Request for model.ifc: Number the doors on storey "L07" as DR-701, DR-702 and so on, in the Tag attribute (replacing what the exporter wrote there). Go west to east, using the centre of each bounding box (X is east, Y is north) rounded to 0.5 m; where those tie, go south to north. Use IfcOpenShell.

First a look at what the model holds.

```python
import ifcopenshell
import ifcopenshell.util.element
import ifcopenshell.util.placement

model = ifcopenshell.open("model.ifc")
print(model.schema)
storey = next(s for s in model.by_type("IfcBuildingStorey") if s.Name == "L07")
doors = [e for e in ifcopenshell.util.element.get_decomposition(storey) if e.is_a("IfcDoor")]
for e in sorted(doors, key=lambda e: e.id()):
    origin = ifcopenshell.util.placement.get_local_placement(e.ObjectPlacement)[:3, 3]
    print(e.id(), e.Tag, e.Name, origin.round(2) + 0.0, sep=" | ")
```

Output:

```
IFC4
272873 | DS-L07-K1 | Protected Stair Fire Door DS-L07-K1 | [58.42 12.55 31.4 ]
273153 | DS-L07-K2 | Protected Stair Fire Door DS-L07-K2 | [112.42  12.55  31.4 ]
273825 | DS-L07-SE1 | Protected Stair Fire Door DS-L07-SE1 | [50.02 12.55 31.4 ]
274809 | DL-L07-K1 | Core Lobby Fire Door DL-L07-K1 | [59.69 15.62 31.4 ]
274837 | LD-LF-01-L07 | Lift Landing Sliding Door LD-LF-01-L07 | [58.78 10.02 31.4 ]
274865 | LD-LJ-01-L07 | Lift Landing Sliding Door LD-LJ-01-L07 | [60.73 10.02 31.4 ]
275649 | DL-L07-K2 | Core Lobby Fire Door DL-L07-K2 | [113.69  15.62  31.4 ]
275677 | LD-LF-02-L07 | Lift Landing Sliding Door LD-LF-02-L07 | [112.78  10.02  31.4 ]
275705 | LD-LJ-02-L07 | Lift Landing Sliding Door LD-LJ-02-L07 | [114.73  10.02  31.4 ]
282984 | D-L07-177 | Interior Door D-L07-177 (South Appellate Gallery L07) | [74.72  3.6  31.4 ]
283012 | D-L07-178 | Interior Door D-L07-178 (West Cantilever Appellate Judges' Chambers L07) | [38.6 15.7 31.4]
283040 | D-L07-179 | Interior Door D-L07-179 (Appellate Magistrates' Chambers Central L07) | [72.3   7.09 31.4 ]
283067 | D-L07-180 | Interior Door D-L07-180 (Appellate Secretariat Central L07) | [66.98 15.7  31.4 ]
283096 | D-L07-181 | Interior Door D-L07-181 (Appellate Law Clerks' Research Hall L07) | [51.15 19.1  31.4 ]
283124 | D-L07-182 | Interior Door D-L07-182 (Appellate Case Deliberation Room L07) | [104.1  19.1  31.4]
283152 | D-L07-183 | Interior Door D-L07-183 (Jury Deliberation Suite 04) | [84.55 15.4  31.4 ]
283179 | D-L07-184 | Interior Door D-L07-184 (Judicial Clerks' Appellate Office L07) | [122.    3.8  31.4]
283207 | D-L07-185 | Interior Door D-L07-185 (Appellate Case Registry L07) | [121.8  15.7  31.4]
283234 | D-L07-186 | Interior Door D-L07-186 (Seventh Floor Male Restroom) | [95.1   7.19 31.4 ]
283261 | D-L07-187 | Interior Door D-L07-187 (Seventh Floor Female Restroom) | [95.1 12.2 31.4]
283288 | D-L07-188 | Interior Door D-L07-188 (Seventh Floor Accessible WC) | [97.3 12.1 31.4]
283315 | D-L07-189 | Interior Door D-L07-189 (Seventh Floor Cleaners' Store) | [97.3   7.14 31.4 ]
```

```python
import ifcopenshell
import ifcopenshell.geom
import ifcopenshell.util.element
import ifcopenshell.util.shape

model = ifcopenshell.open("model.ifc")
settings = ifcopenshell.geom.settings()
settings.set("use-world-coords", True)


def centre(element):
    shape = ifcopenshell.geom.create_shape(settings, element)
    return ifcopenshell.util.shape.get_bbox_centroid(shape.geometry)


storey = next(s for s in model.by_type("IfcBuildingStorey") if s.Name == "L07")
doors = [e for e in ifcopenshell.util.element.get_decomposition(storey) if e.is_a("IfcDoor")]

# Insertion points can sit at a corner or the storey origin, so sort by the geometry (in metres).
centres = {e: centre(e) for e in doors}
doors.sort(key=lambda e: (round(centres[e][0] / 0.5), centres[e][1]))

for i, e in enumerate(doors, start=1):
    number = f"DR-7{i:02d}"
    e.Tag = number
    print(e.id(), number)

model.write("model_rev.ifc")
```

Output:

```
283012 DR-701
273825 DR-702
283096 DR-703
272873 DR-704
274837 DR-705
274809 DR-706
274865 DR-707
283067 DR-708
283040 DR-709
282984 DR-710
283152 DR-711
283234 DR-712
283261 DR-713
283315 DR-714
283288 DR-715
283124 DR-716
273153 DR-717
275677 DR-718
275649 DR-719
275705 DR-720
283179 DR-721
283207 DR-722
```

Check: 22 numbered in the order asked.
